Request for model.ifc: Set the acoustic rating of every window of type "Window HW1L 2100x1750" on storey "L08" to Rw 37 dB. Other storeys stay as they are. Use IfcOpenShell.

First a look at what the model holds.

```python
import ifcopenshell
import ifcopenshell.util.element

model = ifcopenshell.open("model.ifc")
print(model.schema)
storey = next(s for s in model.by_type("IfcBuildingStorey") if s.Name == "L08")
windows = [e for e in ifcopenshell.util.element.get_decomposition(storey) if e.is_a("IfcWindow")]
seen = {}
for e in windows:
    element_type = ifcopenshell.util.element.get_type(e)
    key = (element_type.Name if element_type != e and element_type else None, ifcopenshell.util.element.get_pset(e, "Pset_WindowCommon", "AcousticRating"))
    seen[key] = seen.get(key, 0) + 1
for (name, value), count in sorted(seen.items(), key=str):
    print(count, "x", name, "|", value)
```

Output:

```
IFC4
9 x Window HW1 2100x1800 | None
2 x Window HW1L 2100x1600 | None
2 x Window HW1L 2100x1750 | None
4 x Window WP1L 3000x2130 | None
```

```python
import ifcopenshell
import ifcopenshell.api.pset
import ifcopenshell.util.element

model = ifcopenshell.open("model.ifc")

storey = next(s for s in model.by_type("IfcBuildingStorey") if s.Name == "L08")
windows = [e for e in ifcopenshell.util.element.get_decomposition(storey) if e.is_a("IfcWindow")]

count = 0
for e in windows:
    element_type = ifcopenshell.util.element.get_type(e)
    if element_type in (None, e) or element_type.Name != "Window HW1L 2100x1750":
        continue
    found = ifcopenshell.util.element.get_pset(e, "Pset_WindowCommon", should_inherit=False)
    if found:
        pset = model.by_id(found["id"])
        if len(ifcopenshell.util.element.get_elements_by_pset(pset)) > 1:
            pset = ifcopenshell.api.pset.unshare_pset(model, products=[e], pset=pset)[0]
    else:
        pset = ifcopenshell.api.pset.add_pset(model, product=e, name="Pset_WindowCommon")
    ifcopenshell.api.pset.edit_pset(model, pset=pset, properties={"AcousticRating": "Rw 37 dB"})
    count += 1

print(count, "windows updated")

model.write("model_edited.ifc")
```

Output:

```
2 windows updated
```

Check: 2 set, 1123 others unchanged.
